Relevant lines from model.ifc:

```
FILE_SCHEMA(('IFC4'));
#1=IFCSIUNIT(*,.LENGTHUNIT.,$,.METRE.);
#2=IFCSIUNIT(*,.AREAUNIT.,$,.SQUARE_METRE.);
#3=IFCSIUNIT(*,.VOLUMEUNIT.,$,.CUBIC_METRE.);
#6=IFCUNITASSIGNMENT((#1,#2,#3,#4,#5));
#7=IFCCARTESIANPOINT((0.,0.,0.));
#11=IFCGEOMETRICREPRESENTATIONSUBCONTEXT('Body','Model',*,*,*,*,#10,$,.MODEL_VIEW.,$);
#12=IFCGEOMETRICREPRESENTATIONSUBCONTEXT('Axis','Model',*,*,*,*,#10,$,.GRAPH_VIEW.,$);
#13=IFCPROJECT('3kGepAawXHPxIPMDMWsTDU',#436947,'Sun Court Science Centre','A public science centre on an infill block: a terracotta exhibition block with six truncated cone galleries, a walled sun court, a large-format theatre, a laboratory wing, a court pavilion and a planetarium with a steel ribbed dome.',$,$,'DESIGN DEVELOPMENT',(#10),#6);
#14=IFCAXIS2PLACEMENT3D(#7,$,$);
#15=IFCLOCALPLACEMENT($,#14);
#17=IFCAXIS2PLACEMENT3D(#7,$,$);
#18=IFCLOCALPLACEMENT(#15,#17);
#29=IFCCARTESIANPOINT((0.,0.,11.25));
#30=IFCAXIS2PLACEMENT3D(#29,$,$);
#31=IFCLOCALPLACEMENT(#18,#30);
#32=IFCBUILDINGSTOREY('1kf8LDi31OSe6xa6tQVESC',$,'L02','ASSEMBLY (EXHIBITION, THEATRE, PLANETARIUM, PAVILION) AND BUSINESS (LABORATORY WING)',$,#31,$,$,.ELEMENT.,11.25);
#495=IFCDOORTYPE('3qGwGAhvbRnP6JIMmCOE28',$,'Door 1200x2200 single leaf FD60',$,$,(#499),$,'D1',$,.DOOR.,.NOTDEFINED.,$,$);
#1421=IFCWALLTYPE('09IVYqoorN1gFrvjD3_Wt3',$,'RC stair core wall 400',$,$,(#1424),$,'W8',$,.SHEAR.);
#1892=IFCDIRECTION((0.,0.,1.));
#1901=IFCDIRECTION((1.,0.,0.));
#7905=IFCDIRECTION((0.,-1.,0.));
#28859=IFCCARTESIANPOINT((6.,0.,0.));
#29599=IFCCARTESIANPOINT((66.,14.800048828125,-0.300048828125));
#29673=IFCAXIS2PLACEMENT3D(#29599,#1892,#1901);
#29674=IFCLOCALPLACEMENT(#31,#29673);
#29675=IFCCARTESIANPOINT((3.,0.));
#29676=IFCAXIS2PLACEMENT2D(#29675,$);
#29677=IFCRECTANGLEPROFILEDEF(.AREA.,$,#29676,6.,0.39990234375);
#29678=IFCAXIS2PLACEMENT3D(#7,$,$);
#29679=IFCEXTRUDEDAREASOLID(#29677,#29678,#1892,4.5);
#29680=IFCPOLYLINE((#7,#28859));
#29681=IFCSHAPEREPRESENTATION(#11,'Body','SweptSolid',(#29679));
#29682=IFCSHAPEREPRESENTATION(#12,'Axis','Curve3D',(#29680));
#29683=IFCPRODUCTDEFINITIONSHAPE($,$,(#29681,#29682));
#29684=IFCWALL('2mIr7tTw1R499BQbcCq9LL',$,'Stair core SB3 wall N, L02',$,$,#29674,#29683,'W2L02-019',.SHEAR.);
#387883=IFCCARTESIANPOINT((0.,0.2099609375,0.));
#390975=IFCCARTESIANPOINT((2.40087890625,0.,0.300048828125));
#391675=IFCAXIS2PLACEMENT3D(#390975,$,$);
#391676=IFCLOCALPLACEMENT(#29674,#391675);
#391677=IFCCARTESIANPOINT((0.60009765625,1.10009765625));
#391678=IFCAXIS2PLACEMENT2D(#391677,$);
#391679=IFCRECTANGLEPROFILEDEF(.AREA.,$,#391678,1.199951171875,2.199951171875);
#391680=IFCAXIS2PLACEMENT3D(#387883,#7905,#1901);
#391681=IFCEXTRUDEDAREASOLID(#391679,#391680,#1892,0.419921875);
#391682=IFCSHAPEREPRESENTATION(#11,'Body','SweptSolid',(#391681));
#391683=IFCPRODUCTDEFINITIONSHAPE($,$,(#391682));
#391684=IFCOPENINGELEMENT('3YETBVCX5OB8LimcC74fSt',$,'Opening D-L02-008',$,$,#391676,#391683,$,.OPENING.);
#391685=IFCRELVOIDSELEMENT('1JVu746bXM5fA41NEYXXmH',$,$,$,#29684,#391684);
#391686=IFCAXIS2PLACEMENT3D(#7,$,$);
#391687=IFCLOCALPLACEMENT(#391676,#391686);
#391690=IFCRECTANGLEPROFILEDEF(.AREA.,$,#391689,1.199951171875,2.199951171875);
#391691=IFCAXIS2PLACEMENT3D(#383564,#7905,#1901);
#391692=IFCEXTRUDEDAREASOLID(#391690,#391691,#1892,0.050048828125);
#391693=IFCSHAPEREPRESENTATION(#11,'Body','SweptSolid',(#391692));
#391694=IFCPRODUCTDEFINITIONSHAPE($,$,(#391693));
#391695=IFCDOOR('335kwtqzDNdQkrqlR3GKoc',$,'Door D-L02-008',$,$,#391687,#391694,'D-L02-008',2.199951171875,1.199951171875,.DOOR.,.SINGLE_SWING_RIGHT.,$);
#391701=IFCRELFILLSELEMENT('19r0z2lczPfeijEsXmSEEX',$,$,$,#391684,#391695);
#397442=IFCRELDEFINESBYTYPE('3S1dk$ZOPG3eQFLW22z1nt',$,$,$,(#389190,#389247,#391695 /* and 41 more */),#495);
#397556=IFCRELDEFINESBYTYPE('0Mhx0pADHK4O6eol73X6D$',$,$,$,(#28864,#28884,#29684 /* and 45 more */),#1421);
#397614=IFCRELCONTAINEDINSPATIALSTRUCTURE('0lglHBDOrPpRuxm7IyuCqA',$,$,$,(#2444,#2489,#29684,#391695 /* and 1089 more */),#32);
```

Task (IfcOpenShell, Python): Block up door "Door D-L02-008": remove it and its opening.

```python
import ifcopenshell
import ifcopenshell.api.feature
import ifcopenshell.api.root
import ifcopenshell.geom
import ifcopenshell.util.shape

model = ifcopenshell.open("model.ifc")
settings = ifcopenshell.geom.settings()


def volume(element):
    """Net volume in cubic metres, openings subtracted."""
    shape = ifcopenshell.geom.create_shape(settings, element)
    return ifcopenshell.util.shape.get_volume(shape.geometry)


door = model.by_guid("335kwtqzDNdQkrqlR3GKoc")
opening = door.FillsVoids[0].RelatingOpeningElement
wall = opening.VoidsElements[0].RelatingBuildingElement
before = volume(wall)

ifcopenshell.api.root.remove_product(model, product=door)
ifcopenshell.api.feature.remove_feature(model, feature=opening)

after = volume(wall)

print(f"wall volume {before:.3f} -> {after:.3f} m3")

model.write("model_edited.ifc")
```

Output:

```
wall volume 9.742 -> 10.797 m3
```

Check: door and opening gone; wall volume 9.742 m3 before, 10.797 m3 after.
